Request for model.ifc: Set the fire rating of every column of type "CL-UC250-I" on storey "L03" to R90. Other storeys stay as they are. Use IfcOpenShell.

First a look at what the model holds.

```python
import ifcopenshell
import ifcopenshell.util.element

model = ifcopenshell.open("model.ifc")
print(model.schema)
storey = next(s for s in model.by_type("IfcBuildingStorey") if s.Name == "L03")
columns = [e for e in ifcopenshell.util.element.get_decomposition(storey) if e.is_a("IfcColumn")]
seen = {}
for e in columns:
    element_type = ifcopenshell.util.element.get_type(e)
    key = (element_type.Name if element_type != e and element_type else None, ifcopenshell.util.element.get_pset(e, "Pset_ColumnCommon", "FireRating"))
    seen[key] = seen.get(key, 0) + 1
for (name, value), count in sorted(seen.items(), key=str):
    print(count, "x", name, "|", value)
```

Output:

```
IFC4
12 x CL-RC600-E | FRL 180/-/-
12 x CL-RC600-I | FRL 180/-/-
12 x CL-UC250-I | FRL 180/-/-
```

```python
import ifcopenshell
import ifcopenshell.api.pset
import ifcopenshell.util.element

model = ifcopenshell.open("model.ifc")

storey = next(s for s in model.by_type("IfcBuildingStorey") if s.Name == "L03")
columns = [e for e in ifcopenshell.util.element.get_decomposition(storey) if e.is_a("IfcColumn")]

count = 0
for e in columns:
    element_type = ifcopenshell.util.element.get_type(e)
    if element_type in (None, e) or element_type.Name != "CL-UC250-I":
        continue
    # add_pset returns the element's existing set when there is one.
    pset = ifcopenshell.api.pset.add_pset(model, product=e, name="Pset_ColumnCommon")
    ifcopenshell.api.pset.edit_pset(model, pset=pset, properties={"FireRating": "R90"})
    count += 1

print(count, "columns updated")

model.write("model_rev.ifc")
```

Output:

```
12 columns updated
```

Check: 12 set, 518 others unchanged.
